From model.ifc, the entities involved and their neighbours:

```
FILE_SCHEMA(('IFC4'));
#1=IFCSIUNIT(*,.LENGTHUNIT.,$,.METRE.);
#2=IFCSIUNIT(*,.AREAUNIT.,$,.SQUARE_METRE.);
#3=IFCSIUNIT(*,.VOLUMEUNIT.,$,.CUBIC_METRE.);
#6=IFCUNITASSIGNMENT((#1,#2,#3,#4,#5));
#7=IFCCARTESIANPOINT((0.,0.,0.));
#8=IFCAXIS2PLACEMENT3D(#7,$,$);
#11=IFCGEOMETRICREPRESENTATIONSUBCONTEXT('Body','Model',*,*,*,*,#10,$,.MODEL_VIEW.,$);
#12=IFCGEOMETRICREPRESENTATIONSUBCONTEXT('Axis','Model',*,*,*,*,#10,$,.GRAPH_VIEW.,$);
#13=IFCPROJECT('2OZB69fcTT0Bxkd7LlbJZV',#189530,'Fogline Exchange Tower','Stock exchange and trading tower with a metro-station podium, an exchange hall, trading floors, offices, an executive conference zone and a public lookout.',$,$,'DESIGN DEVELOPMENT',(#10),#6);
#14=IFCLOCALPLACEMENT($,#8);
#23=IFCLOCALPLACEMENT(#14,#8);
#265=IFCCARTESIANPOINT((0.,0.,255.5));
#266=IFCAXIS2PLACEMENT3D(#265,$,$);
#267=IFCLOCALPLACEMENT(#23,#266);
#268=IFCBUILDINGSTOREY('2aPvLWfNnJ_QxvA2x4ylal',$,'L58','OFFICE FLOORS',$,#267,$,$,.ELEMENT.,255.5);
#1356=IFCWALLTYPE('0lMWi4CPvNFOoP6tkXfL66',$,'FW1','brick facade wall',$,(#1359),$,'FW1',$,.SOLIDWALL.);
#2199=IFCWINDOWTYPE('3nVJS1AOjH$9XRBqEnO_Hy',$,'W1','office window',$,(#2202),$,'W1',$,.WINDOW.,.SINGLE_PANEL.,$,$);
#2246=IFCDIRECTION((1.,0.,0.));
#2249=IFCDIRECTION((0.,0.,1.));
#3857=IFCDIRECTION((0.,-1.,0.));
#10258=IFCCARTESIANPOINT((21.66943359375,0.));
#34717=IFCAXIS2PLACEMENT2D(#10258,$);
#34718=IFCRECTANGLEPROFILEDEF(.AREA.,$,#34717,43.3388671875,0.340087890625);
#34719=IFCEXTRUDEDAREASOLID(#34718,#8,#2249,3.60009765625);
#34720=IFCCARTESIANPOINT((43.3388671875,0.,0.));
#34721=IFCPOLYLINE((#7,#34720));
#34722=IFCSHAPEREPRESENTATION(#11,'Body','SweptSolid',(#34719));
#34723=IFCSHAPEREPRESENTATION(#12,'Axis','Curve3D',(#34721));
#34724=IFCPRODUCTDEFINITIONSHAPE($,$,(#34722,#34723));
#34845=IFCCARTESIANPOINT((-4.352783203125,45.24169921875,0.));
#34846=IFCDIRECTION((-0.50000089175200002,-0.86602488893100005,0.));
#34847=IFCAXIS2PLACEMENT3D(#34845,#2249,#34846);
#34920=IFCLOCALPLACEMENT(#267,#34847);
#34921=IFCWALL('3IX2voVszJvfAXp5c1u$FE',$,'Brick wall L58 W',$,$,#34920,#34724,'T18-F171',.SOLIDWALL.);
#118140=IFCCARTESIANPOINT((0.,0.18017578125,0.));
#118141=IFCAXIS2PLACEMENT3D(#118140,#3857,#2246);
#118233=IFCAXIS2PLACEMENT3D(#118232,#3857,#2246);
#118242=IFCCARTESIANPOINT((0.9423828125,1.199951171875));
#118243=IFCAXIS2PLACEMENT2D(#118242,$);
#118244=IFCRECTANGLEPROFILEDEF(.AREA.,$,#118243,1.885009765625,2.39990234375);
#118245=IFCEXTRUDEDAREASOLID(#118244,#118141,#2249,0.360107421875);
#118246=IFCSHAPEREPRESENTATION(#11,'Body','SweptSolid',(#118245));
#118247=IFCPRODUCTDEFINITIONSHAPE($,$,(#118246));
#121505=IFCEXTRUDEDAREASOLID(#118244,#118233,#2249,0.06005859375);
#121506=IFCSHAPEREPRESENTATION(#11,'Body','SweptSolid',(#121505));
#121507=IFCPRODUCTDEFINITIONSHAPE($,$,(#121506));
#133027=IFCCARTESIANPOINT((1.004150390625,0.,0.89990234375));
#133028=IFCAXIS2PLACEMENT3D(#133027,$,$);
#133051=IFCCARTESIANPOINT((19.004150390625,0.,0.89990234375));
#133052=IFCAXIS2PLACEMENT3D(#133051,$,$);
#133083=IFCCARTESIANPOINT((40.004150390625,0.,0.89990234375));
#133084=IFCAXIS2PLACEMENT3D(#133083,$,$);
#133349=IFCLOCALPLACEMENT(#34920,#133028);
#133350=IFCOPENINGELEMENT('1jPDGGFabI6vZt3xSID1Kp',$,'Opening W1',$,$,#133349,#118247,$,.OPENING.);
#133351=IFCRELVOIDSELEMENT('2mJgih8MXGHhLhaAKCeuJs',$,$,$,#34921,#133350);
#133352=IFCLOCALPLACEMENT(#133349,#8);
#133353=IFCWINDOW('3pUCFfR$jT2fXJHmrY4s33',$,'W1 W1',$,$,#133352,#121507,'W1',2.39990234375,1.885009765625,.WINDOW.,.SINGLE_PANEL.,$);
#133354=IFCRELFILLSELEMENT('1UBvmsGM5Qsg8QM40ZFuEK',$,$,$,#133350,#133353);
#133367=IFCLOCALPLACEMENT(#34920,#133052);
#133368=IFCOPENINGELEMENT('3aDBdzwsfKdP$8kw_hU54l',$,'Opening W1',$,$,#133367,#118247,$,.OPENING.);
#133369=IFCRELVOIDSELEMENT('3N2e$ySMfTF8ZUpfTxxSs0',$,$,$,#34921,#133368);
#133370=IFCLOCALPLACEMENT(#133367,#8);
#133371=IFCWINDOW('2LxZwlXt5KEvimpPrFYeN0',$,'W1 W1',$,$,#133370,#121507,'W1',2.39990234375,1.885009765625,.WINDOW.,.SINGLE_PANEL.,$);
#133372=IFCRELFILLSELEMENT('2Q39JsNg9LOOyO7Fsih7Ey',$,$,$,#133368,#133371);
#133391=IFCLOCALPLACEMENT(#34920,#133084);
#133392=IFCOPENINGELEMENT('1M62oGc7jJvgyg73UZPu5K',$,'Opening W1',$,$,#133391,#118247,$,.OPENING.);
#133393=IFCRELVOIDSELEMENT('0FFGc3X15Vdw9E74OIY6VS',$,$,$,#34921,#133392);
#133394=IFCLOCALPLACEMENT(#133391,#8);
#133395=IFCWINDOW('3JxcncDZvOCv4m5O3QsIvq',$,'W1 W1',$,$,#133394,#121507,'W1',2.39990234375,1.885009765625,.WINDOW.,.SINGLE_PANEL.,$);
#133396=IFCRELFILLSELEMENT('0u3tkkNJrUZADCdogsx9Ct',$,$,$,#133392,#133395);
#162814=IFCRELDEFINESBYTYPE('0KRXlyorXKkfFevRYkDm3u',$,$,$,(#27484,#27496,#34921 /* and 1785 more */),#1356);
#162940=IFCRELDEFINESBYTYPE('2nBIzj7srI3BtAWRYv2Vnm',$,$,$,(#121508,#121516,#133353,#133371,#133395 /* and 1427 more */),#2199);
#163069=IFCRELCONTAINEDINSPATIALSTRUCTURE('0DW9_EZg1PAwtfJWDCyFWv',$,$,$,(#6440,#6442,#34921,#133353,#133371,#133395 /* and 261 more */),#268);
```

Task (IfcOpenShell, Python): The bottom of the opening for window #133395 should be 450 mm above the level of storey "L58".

```python
import numpy as np
import ifcopenshell
import ifcopenshell.api.geometry
import ifcopenshell.geom
import ifcopenshell.util.element
import ifcopenshell.util.placement
import ifcopenshell.util.shape
import ifcopenshell.util.unit

model = ifcopenshell.open("model.ifc")
unit_scale = ifcopenshell.util.unit.calculate_unit_scale(model)

window = model.by_guid("3JxcncDZvOCv4m5O3QsIvq")
opening = window.FillsVoids[0].RelatingOpeningElement
storey = ifcopenshell.util.element.get_container(window, ifc_class="IfcBuildingStorey")
level = ifcopenshell.util.placement.get_local_placement(storey.ObjectPlacement)[2, 3]

# The opening's origin need not be at the sill, so measure its lowest point.
shape = ifcopenshell.geom.create_shape(ifcopenshell.geom.settings(), opening)
bottom = ifcopenshell.util.shape.get_shape_bottom_elevation(shape, shape.geometry) / unit_scale
dz = level + 0.45 / unit_scale - bottom

shift = np.array([0.0, 0.0, dz])
# The window is placed relative to its opening, so it follows when the opening moves.
matrix = ifcopenshell.util.placement.get_local_placement(opening.ObjectPlacement)
matrix[:3, 3] += shift
ifcopenshell.api.geometry.edit_object_placement(
    model, product=opening, matrix=matrix, is_si=False, should_transform_children=True
)

print(f"moved by {dz * unit_scale:+.3f} m")

model.write("model_updated.ifc")
```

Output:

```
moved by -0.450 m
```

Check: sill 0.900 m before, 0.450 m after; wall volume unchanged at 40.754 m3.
